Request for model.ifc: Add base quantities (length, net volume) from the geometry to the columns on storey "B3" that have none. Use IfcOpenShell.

First a look at what the model holds.

```python
import ifcopenshell
import ifcopenshell.util.element
import ifcopenshell.util.unit

model = ifcopenshell.open("model.ifc")
print(model.schema)
for unit_type in ("LENGTHUNIT", "AREAUNIT", "VOLUMEUNIT"):
    print(unit_type, ifcopenshell.util.unit.calculate_unit_scale(model, unit_type))
storey = next(s for s in model.by_type("IfcBuildingStorey") if s.Name == "B3")
columns = [e for e in ifcopenshell.util.element.get_decomposition(storey) if e.is_a("IfcColumn")]
for e in sorted(columns, key=lambda e: e.id()):
    print(e.id(), e.is_a(), e.Name, list(ifcopenshell.util.element.get_psets(e, qtos_only=True)), sep=" | ")
```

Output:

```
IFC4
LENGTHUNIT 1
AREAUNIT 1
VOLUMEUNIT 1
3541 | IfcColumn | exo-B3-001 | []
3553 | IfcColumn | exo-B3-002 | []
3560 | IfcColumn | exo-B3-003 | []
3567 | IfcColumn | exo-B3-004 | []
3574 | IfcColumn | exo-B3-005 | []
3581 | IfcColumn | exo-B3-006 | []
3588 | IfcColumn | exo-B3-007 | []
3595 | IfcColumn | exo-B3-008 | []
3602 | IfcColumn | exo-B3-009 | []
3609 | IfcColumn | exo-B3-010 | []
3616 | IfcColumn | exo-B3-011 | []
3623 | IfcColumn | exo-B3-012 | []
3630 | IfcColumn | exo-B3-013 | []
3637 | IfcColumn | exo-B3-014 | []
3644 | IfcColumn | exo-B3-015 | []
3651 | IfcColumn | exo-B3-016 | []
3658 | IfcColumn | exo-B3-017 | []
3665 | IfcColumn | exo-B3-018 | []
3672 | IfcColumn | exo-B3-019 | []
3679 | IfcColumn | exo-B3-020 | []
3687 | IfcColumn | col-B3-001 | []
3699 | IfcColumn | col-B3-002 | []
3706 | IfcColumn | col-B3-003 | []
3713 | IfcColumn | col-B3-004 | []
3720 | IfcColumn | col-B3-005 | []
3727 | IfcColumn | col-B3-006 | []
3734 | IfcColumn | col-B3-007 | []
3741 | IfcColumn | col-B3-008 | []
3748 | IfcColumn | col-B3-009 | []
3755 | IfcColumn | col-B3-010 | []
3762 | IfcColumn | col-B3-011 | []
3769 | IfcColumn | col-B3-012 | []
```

```python
import ifcopenshell
import ifcopenshell.api.pset
import ifcopenshell.geom
import ifcopenshell.util.element
import ifcopenshell.util.shape
import ifcopenshell.util.unit

model = ifcopenshell.open("model.ifc")
unit_scale = ifcopenshell.util.unit.calculate_unit_scale(model)
volume_scale = ifcopenshell.util.unit.calculate_unit_scale(model, "VOLUMEUNIT")
settings = ifcopenshell.geom.settings()

storey = next(s for s in model.by_type("IfcBuildingStorey") if s.Name == "B3")
columns = [e for e in ifcopenshell.util.element.get_decomposition(storey) if e.is_a("IfcColumn")]

for e in sorted(columns, key=lambda e: e.id()):
    if ifcopenshell.util.element.get_psets(e, qtos_only=True, should_inherit=False):
        continue
    # Geometry comes back in metres, in the element's own axes.
    shape = ifcopenshell.geom.create_shape(settings, e)
    values = {
        "Length": ifcopenshell.util.shape.get_z(shape.geometry) / unit_scale,
        "NetVolume": ifcopenshell.util.shape.get_volume(shape.geometry) / volume_scale,
    }
    qto = ifcopenshell.api.pset.add_qto(model, product=e, name="Qto_ColumnBaseQuantities")
    ifcopenshell.api.pset.edit_qto(model, qto=qto, properties=values)
    print(e.id(), {k: round(v, 3) for k, v in values.items()})

model.write("model_edited.ifc")
```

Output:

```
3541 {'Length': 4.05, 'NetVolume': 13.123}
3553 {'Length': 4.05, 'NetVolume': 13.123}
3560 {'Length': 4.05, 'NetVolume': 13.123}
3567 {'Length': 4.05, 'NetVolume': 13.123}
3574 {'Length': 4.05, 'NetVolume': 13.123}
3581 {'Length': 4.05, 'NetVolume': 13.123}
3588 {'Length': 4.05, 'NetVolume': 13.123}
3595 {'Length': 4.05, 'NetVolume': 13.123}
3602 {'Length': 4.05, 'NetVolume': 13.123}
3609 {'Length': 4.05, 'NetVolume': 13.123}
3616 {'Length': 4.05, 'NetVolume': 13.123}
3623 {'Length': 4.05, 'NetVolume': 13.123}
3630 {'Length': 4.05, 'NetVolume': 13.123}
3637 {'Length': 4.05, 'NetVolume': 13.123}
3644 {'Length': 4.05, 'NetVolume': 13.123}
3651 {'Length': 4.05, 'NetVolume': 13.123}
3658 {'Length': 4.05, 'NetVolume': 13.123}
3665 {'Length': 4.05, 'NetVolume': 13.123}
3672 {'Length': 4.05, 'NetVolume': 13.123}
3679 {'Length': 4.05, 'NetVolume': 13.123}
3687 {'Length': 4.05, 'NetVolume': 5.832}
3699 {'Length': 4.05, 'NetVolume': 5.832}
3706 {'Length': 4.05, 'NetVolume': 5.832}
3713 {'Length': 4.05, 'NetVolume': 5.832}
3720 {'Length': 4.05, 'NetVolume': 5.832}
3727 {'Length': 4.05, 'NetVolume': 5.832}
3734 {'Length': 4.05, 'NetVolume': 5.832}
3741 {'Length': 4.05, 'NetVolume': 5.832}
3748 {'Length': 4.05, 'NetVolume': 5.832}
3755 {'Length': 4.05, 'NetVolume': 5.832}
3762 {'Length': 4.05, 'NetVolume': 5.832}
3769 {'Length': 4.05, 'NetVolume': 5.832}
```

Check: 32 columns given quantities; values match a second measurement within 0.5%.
